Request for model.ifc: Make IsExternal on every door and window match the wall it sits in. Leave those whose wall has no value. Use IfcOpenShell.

First a look at what the model holds.

```python
import ifcopenshell
import ifcopenshell.util.element

model = ifcopenshell.open("model.ifc")
print(model.schema)
seen = {}
for e in model.by_type("IfcDoor") + model.by_type("IfcWindow"):
    if not e.FillsVoids:
        continue
    host = e.FillsVoids[0].RelatingOpeningElement.VoidsElements[0].RelatingBuildingElement
    own = ifcopenshell.util.element.get_pset(e, f"Pset_{e.is_a()[3:].removesuffix('StandardCase')}Common", "IsExternal")
    wall = ifcopenshell.util.element.get_pset(host, "Pset_WallCommon", "IsExternal")
    seen[e.is_a(), own, wall] = seen.get((e.is_a(), own, wall), 0) + 1
for (cls, own, wall), count in sorted(seen.items(), key=str):
    print(count, cls, "IsExternal:", own, "| host wall:", wall)
```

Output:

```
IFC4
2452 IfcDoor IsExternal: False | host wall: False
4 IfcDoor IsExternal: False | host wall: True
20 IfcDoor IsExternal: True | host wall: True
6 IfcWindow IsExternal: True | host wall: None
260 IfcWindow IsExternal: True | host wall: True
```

```python
import ifcopenshell
import ifcopenshell.api.pset
import ifcopenshell.util.element

model = ifcopenshell.open("model.ifc")

count = 0
for ifc_class, pset_name in (("IfcDoor", "Pset_DoorCommon"), ("IfcWindow", "Pset_WindowCommon")):
    for e in model.by_type(ifc_class):
        if not e.FillsVoids:
            continue
        host = e.FillsVoids[0].RelatingOpeningElement.VoidsElements[0].RelatingBuildingElement
        external = ifcopenshell.util.element.get_pset(host, "Pset_WallCommon", "IsExternal")
        if external is None or ifcopenshell.util.element.get_pset(e, pset_name, "IsExternal") == external:
            continue
        pset = ifcopenshell.api.pset.add_pset(model, product=e, name=pset_name)
        ifcopenshell.api.pset.edit_pset(model, pset=pset, properties={"IsExternal": external})
        count += 1

print(count, "updated")

model.write("model_rev.ifc")
```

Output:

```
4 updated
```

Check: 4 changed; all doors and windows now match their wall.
